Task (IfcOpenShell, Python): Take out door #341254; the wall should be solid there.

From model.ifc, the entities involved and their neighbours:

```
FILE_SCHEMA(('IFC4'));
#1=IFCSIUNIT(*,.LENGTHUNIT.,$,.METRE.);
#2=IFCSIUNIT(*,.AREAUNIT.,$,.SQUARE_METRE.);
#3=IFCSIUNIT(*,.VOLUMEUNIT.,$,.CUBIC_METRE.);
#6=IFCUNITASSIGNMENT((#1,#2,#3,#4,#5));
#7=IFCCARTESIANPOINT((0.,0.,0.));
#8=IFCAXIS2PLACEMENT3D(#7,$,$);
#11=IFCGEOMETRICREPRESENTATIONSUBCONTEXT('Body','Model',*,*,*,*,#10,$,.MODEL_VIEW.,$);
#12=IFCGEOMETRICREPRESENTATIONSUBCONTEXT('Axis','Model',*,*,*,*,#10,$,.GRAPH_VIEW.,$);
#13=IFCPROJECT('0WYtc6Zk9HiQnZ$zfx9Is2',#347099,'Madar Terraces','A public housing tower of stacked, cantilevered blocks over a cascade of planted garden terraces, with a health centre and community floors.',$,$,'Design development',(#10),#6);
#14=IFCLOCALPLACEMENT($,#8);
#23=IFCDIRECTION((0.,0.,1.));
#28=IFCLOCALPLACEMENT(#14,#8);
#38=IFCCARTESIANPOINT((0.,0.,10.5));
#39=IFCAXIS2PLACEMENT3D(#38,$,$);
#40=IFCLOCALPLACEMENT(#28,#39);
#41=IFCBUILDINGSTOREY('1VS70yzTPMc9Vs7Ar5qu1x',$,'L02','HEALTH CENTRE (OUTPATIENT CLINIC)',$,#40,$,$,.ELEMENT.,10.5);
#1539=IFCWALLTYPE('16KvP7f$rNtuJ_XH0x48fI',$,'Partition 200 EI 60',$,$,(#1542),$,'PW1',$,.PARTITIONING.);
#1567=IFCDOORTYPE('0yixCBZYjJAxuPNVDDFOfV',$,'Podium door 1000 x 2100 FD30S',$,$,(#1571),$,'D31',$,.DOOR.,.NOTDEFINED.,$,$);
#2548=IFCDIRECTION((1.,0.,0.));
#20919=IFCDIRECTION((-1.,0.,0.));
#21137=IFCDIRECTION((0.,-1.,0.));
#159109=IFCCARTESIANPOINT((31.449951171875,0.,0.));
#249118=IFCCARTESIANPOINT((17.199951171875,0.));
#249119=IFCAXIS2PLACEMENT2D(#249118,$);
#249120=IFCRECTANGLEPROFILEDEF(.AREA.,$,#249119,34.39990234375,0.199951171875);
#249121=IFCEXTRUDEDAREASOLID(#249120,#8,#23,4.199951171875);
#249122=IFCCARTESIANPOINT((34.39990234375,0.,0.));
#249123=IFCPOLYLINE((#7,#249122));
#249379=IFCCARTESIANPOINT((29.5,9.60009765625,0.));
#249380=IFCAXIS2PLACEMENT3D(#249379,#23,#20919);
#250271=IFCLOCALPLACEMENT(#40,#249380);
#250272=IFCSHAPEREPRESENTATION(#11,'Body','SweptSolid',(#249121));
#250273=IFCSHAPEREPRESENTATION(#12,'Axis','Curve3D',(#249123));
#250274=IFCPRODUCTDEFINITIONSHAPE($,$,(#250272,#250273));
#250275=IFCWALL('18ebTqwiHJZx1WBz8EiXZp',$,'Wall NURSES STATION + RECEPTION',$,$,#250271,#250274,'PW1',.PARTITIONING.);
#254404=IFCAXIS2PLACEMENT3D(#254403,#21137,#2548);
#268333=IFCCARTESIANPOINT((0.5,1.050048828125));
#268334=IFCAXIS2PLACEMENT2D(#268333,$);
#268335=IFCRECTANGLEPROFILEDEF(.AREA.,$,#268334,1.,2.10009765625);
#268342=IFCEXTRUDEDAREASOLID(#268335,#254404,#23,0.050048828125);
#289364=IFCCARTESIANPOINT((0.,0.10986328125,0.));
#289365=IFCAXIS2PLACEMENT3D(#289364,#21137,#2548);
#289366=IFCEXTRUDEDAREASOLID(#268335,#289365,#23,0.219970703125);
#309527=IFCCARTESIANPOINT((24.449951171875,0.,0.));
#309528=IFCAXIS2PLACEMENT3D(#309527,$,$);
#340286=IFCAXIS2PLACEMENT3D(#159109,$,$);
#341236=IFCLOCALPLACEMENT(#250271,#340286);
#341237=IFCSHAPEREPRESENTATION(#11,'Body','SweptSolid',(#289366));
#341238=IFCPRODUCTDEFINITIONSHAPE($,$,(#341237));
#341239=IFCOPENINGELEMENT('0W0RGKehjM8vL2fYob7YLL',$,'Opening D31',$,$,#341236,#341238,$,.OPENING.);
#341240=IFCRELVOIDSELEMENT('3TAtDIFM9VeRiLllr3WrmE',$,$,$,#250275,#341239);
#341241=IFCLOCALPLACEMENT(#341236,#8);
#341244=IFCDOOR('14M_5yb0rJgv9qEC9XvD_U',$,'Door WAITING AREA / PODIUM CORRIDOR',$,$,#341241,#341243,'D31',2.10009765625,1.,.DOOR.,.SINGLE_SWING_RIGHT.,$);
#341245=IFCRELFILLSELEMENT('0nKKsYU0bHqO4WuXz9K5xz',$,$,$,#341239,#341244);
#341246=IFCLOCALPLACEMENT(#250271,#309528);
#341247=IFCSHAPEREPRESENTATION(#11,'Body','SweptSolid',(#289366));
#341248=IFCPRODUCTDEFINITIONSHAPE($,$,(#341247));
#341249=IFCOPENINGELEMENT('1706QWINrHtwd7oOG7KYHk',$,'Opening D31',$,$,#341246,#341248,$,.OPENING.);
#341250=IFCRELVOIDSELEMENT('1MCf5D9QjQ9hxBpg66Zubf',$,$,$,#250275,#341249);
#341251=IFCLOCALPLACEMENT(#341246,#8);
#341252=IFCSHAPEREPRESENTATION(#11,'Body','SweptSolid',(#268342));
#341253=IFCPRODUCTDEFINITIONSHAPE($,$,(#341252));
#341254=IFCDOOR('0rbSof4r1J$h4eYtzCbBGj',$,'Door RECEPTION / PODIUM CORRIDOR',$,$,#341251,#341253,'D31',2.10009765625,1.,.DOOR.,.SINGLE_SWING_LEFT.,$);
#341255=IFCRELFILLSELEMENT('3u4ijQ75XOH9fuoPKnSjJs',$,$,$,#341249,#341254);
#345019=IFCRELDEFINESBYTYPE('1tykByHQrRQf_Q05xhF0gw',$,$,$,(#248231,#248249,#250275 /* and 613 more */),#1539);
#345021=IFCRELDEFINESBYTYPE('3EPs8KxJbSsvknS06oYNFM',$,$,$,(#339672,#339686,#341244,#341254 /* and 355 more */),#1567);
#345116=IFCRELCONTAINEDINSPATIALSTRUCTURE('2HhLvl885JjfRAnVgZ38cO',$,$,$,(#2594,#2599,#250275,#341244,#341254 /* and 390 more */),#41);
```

```python
import ifcopenshell
import ifcopenshell.api.feature
import ifcopenshell.api.root
import ifcopenshell.geom
import ifcopenshell.util.shape

model = ifcopenshell.open("model.ifc")
settings = ifcopenshell.geom.settings()


def volume(element):
    """Net volume in cubic metres, openings subtracted."""
    shape = ifcopenshell.geom.create_shape(settings, element)
    return ifcopenshell.util.shape.get_volume(shape.geometry)


door = model.by_guid("0rbSof4r1J$h4eYtzCbBGj")
opening = door.FillsVoids[0].RelatingOpeningElement
wall = opening.VoidsElements[0].RelatingBuildingElement
before = volume(wall)

ifcopenshell.api.root.remove_product(model, product=door)
ifcopenshell.api.feature.remove_feature(model, feature=opening)

after = volume(wall)

print(f"wall volume {before:.3f} -> {after:.3f} m3")

model.write("model_v2.ifc")
```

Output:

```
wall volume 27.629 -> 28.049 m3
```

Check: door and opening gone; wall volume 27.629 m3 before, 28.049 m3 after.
